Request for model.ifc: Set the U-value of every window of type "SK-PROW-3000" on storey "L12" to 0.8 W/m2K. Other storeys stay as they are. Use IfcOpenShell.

First a look at what the model holds.

```python
import ifcopenshell
import ifcopenshell.util.element

model = ifcopenshell.open("model.ifc")
print(model.schema)
storey = next(s for s in model.by_type("IfcBuildingStorey") if s.Name == "L12")
windows = [e for e in ifcopenshell.util.element.get_decomposition(storey) if e.is_a("IfcWindow")]
seen = {}
for e in windows:
    element_type = ifcopenshell.util.element.get_type(e)
    key = (element_type.Name if element_type != e and element_type else None, ifcopenshell.util.element.get_pset(e, "Pset_WindowCommon", "ThermalTransmittance"))
    seen[key] = seen.get(key, 0) + 1
for (name, value), count in sorted(seen.items(), key=str):
    print(count, "x", name, "|", value)
```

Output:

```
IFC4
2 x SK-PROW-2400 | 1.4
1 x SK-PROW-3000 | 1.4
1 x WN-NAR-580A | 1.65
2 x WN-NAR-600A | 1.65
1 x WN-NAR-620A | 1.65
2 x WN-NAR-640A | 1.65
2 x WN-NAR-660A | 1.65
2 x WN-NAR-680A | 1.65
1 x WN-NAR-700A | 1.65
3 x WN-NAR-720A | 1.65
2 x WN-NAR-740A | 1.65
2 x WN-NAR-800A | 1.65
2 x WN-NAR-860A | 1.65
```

```python
import ifcopenshell
import ifcopenshell.api.pset
import ifcopenshell.util.element

model = ifcopenshell.open("model.ifc")

storey = next(s for s in model.by_type("IfcBuildingStorey") if s.Name == "L12")
windows = [e for e in ifcopenshell.util.element.get_decomposition(storey) if e.is_a("IfcWindow")]

count = 0
for e in windows:
    element_type = ifcopenshell.util.element.get_type(e)
    if element_type in (None, e) or element_type.Name != "SK-PROW-3000":
        continue
    # add_pset returns the element's existing set when there is one.
    pset = ifcopenshell.api.pset.add_pset(model, product=e, name="Pset_WindowCommon")
    ifcopenshell.api.pset.edit_pset(model, pset=pset, properties={"ThermalTransmittance": 0.8})
    count += 1

print(count, "windows updated")

model.write("model-out.ifc")
```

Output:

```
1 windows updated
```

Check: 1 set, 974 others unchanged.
